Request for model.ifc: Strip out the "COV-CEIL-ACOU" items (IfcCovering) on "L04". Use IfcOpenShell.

First a look at what the model holds.

```python
import ifcopenshell
import ifcopenshell.util.element

model = ifcopenshell.open("model.ifc")
print(model.schema)
storey = next(s for s in model.by_type("IfcBuildingStorey") if s.Name == "L04")
coverings = [e for e in ifcopenshell.util.element.get_decomposition(storey) if e.is_a("IfcCovering")]
seen = {}
for e in coverings:
    element_type = ifcopenshell.util.element.get_type(e)
    name = element_type.Name if element_type not in (None, e) else None
    seen[name] = seen.get(name, 0) + 1
for name, count in sorted(seen.items(), key=str):
    print(count, "x", name)
```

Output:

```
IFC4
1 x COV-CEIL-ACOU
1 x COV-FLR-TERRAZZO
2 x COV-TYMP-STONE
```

```python
import ifcopenshell
import ifcopenshell.api.root
import ifcopenshell.util.element

model = ifcopenshell.open("model.ifc")

storey = next(s for s in model.by_type("IfcBuildingStorey") if s.Name == "L04")
coverings = [e for e in ifcopenshell.util.element.get_decomposition(storey) if e.is_a("IfcCovering")]
targets = [e for e in coverings if (t := ifcopenshell.util.element.get_type(e)) not in (None, e) and t.Name == "COV-CEIL-ACOU"]

for e in targets:
    ifcopenshell.api.root.remove_product(model, product=e)
print(len(targets), "removed")

model.write("model-out.ifc")
```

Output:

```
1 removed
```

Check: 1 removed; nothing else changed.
